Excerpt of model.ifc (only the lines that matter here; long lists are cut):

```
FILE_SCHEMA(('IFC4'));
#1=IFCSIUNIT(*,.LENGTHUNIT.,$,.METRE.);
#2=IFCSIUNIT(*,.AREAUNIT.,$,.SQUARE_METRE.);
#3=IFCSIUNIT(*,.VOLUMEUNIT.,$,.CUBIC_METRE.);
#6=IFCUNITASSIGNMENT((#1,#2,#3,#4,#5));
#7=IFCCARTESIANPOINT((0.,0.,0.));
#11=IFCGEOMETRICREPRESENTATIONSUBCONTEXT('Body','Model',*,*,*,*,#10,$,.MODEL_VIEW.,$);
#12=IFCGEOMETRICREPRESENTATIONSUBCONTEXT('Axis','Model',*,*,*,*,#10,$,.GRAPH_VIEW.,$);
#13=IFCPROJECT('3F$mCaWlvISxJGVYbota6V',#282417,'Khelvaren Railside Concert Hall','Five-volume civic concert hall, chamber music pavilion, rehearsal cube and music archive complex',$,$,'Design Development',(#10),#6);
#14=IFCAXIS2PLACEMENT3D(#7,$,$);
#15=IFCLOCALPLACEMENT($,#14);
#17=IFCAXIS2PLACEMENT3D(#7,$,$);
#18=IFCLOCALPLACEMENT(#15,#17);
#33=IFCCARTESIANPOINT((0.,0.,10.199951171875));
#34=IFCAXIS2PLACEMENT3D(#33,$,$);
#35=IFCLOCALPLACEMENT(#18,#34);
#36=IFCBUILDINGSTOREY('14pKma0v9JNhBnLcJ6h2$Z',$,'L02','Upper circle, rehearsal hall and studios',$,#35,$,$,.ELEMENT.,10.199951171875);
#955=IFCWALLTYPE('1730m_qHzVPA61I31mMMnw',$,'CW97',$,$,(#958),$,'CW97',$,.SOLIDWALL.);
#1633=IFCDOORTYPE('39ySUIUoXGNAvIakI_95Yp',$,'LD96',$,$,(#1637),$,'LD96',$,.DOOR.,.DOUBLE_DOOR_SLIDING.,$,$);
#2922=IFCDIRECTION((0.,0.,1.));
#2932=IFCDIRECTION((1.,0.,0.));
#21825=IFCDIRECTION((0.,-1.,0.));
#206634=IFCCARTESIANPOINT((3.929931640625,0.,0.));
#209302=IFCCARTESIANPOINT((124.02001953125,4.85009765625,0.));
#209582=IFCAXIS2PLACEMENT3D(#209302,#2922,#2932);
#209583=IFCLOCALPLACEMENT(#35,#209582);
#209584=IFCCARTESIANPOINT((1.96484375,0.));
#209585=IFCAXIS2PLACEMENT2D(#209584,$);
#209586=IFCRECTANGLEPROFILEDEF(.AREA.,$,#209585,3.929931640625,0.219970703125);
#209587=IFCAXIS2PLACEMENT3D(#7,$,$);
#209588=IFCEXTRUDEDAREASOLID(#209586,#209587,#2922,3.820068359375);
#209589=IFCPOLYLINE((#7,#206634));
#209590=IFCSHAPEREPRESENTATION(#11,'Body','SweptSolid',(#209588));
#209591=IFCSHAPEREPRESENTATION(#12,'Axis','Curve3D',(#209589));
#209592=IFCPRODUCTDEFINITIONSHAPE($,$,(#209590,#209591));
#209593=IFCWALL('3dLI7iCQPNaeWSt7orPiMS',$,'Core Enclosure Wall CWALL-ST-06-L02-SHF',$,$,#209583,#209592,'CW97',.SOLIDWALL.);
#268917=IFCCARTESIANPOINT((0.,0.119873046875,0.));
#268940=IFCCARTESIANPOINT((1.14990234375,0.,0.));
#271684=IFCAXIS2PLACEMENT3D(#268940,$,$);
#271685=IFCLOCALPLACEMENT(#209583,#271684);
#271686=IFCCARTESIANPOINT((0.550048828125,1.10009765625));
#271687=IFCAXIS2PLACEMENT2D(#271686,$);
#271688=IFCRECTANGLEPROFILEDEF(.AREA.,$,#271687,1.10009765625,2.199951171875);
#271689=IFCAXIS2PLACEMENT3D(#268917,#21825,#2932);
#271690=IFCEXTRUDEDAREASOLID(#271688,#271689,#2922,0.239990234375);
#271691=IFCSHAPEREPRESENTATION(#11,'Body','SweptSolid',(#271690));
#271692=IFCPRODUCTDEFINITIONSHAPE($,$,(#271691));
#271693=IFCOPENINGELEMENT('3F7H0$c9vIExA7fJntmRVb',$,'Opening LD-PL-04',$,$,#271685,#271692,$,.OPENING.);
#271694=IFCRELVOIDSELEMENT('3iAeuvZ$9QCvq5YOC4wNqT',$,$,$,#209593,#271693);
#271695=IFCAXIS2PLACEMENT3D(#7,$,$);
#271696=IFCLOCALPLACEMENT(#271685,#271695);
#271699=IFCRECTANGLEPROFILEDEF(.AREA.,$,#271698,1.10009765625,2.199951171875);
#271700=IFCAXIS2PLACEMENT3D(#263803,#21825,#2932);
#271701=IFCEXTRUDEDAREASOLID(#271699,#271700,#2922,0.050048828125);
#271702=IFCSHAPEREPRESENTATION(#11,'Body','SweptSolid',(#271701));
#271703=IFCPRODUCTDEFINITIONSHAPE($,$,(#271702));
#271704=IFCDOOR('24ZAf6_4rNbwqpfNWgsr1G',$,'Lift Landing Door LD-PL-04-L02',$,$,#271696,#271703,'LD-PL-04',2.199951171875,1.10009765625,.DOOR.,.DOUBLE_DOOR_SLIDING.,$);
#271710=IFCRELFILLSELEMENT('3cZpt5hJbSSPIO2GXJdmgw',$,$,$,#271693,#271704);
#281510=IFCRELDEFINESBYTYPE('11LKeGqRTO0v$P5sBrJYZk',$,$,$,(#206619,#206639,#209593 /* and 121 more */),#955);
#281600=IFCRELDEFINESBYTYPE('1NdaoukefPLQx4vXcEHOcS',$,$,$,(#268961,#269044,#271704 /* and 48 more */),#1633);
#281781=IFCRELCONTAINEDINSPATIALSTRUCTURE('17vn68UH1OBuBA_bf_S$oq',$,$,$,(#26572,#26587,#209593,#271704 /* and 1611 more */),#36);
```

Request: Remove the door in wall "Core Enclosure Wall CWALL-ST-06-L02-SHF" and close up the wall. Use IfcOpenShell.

```python
import ifcopenshell
import ifcopenshell.api.feature
import ifcopenshell.api.root
import ifcopenshell.geom
import ifcopenshell.util.shape

model = ifcopenshell.open("model.ifc")
settings = ifcopenshell.geom.settings()


def volume(element):
    """Net volume in cubic metres, openings subtracted."""
    shape = ifcopenshell.geom.create_shape(settings, element)
    return ifcopenshell.util.shape.get_volume(shape.geometry)


door = model.by_id(271704)
opening = door.FillsVoids[0].RelatingOpeningElement
wall = opening.VoidsElements[0].RelatingBuildingElement
before = volume(wall)

ifcopenshell.api.root.remove_product(model, product=door)
ifcopenshell.api.feature.remove_feature(model, feature=opening)

after = volume(wall)

print(f"wall volume {before:.3f} -> {after:.3f} m3")

model.write("model_v2.ifc")
```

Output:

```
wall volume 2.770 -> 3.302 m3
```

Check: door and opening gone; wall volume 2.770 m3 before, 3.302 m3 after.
